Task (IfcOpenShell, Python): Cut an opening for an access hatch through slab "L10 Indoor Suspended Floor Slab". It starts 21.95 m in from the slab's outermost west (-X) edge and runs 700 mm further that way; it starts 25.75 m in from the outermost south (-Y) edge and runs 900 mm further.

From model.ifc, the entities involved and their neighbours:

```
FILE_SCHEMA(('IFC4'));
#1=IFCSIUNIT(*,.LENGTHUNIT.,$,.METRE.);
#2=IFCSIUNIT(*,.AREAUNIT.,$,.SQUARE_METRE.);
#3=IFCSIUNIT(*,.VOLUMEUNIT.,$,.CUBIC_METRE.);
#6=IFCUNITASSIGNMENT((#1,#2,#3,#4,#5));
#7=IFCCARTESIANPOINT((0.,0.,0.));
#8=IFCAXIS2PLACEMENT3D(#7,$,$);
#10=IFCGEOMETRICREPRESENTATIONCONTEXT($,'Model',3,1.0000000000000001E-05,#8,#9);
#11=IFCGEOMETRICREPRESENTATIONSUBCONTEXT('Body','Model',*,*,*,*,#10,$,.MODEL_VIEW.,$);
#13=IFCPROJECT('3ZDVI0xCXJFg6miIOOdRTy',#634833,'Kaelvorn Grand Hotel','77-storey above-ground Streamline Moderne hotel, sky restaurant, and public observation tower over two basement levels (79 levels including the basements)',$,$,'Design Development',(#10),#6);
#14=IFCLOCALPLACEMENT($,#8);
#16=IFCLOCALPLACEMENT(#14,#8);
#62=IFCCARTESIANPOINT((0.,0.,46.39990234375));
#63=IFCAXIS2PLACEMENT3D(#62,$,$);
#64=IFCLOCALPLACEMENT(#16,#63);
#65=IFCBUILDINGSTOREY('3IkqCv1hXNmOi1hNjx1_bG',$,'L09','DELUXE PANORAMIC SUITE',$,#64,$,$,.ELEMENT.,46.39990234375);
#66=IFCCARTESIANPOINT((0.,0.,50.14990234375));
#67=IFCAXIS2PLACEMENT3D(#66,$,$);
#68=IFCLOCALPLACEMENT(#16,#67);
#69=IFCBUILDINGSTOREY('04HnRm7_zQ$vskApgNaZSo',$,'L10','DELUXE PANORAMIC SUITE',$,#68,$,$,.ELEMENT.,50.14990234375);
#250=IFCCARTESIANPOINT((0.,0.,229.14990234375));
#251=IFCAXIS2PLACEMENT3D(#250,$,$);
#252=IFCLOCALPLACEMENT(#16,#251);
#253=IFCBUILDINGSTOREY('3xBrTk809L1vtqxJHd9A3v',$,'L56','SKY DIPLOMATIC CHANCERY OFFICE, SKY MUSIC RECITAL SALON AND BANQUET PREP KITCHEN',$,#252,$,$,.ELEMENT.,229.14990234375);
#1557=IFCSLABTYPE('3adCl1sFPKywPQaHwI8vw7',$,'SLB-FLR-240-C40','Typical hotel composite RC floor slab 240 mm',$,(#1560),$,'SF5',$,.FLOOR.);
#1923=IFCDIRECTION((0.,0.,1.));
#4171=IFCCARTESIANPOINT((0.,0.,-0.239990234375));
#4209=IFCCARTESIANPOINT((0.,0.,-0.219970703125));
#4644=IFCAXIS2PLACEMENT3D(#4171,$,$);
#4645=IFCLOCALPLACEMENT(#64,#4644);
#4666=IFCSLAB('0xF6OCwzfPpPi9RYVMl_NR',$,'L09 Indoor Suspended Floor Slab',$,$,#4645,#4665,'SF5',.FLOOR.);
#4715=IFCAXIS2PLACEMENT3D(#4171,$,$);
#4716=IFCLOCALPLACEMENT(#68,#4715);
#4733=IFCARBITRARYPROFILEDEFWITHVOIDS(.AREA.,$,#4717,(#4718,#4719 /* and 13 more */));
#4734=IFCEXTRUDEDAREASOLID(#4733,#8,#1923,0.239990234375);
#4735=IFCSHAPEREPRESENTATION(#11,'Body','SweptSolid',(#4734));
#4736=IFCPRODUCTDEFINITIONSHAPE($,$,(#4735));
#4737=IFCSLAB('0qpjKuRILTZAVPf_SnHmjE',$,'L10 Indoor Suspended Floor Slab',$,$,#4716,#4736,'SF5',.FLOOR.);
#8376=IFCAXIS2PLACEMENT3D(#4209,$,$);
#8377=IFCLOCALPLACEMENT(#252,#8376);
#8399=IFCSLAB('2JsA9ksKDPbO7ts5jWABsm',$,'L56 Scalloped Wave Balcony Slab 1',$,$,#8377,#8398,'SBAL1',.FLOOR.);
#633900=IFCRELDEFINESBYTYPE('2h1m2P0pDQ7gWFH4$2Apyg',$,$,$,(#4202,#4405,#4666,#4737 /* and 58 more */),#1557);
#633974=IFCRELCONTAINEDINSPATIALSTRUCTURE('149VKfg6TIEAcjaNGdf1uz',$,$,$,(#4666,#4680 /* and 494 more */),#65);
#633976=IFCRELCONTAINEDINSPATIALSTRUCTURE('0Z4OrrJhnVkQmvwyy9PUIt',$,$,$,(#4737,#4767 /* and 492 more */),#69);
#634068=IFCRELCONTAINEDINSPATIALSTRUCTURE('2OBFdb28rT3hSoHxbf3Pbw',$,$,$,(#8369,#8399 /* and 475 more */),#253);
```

```python
import numpy as np
import ifcopenshell
import ifcopenshell.api.feature
import ifcopenshell.api.geometry
import ifcopenshell.api.root
import ifcopenshell.geom
import ifcopenshell.util.placement
import ifcopenshell.util.representation
import ifcopenshell.util.shape
import ifcopenshell.util.unit

model = ifcopenshell.open("model.ifc")
unit_scale = ifcopenshell.util.unit.calculate_unit_scale(model)
settings = ifcopenshell.geom.settings()


def volume(element):
    """Net volume in cubic metres, openings subtracted."""
    shape = ifcopenshell.geom.create_shape(settings, element)
    return ifcopenshell.util.shape.get_volume(shape.geometry)


slab = model.by_id(4737)
before = volume(slab)

# Extent in the slab's own axes, in metres. The edges named are its -X and -Y sides.
slab_shape = ifcopenshell.geom.create_shape(settings, slab)
vertices = ifcopenshell.util.shape.get_vertices(slab_shape.geometry)
x_min, y_min, bottom = vertices.min(axis=0)
top = vertices[:, 2].max()

opening = ifcopenshell.api.root.create_entity(model, ifc_class="IfcOpeningElement", name="Access hatch opening", predefined_type="OPENING")
context = ifcopenshell.util.representation.get_context(model, "Model", "Body", "MODEL_VIEW")
width, depth = 0.7, 0.9
outline = [(0.0, 0.0), (width, 0.0), (width, depth), (0.0, depth), (0.0, 0.0)]
# Overshoot both faces by 50 mm so the cut is clean.
shape = ifcopenshell.api.geometry.add_slab_representation(
    model, context=context, depth=top - bottom + 0.1, polyline=outline
)
ifcopenshell.api.geometry.assign_representation(model, product=opening, representation=shape)

matrix = ifcopenshell.util.placement.get_local_placement(slab.ObjectPlacement)
matrix[:, 3] = matrix @ np.append(np.array([x_min + 21.95, y_min + 25.75, bottom - 0.05]) / unit_scale, 1.0)
ifcopenshell.api.geometry.edit_object_placement(model, product=opening, matrix=matrix, is_si=False)
ifcopenshell.api.feature.add_feature(model, feature=opening, element=slab)

after = volume(slab)

print(f"slab volume {before:.3f} -> {after:.3f} m3")

model.write("model_updated.ifc")
```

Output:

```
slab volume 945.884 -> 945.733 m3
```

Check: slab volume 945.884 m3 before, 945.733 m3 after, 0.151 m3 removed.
